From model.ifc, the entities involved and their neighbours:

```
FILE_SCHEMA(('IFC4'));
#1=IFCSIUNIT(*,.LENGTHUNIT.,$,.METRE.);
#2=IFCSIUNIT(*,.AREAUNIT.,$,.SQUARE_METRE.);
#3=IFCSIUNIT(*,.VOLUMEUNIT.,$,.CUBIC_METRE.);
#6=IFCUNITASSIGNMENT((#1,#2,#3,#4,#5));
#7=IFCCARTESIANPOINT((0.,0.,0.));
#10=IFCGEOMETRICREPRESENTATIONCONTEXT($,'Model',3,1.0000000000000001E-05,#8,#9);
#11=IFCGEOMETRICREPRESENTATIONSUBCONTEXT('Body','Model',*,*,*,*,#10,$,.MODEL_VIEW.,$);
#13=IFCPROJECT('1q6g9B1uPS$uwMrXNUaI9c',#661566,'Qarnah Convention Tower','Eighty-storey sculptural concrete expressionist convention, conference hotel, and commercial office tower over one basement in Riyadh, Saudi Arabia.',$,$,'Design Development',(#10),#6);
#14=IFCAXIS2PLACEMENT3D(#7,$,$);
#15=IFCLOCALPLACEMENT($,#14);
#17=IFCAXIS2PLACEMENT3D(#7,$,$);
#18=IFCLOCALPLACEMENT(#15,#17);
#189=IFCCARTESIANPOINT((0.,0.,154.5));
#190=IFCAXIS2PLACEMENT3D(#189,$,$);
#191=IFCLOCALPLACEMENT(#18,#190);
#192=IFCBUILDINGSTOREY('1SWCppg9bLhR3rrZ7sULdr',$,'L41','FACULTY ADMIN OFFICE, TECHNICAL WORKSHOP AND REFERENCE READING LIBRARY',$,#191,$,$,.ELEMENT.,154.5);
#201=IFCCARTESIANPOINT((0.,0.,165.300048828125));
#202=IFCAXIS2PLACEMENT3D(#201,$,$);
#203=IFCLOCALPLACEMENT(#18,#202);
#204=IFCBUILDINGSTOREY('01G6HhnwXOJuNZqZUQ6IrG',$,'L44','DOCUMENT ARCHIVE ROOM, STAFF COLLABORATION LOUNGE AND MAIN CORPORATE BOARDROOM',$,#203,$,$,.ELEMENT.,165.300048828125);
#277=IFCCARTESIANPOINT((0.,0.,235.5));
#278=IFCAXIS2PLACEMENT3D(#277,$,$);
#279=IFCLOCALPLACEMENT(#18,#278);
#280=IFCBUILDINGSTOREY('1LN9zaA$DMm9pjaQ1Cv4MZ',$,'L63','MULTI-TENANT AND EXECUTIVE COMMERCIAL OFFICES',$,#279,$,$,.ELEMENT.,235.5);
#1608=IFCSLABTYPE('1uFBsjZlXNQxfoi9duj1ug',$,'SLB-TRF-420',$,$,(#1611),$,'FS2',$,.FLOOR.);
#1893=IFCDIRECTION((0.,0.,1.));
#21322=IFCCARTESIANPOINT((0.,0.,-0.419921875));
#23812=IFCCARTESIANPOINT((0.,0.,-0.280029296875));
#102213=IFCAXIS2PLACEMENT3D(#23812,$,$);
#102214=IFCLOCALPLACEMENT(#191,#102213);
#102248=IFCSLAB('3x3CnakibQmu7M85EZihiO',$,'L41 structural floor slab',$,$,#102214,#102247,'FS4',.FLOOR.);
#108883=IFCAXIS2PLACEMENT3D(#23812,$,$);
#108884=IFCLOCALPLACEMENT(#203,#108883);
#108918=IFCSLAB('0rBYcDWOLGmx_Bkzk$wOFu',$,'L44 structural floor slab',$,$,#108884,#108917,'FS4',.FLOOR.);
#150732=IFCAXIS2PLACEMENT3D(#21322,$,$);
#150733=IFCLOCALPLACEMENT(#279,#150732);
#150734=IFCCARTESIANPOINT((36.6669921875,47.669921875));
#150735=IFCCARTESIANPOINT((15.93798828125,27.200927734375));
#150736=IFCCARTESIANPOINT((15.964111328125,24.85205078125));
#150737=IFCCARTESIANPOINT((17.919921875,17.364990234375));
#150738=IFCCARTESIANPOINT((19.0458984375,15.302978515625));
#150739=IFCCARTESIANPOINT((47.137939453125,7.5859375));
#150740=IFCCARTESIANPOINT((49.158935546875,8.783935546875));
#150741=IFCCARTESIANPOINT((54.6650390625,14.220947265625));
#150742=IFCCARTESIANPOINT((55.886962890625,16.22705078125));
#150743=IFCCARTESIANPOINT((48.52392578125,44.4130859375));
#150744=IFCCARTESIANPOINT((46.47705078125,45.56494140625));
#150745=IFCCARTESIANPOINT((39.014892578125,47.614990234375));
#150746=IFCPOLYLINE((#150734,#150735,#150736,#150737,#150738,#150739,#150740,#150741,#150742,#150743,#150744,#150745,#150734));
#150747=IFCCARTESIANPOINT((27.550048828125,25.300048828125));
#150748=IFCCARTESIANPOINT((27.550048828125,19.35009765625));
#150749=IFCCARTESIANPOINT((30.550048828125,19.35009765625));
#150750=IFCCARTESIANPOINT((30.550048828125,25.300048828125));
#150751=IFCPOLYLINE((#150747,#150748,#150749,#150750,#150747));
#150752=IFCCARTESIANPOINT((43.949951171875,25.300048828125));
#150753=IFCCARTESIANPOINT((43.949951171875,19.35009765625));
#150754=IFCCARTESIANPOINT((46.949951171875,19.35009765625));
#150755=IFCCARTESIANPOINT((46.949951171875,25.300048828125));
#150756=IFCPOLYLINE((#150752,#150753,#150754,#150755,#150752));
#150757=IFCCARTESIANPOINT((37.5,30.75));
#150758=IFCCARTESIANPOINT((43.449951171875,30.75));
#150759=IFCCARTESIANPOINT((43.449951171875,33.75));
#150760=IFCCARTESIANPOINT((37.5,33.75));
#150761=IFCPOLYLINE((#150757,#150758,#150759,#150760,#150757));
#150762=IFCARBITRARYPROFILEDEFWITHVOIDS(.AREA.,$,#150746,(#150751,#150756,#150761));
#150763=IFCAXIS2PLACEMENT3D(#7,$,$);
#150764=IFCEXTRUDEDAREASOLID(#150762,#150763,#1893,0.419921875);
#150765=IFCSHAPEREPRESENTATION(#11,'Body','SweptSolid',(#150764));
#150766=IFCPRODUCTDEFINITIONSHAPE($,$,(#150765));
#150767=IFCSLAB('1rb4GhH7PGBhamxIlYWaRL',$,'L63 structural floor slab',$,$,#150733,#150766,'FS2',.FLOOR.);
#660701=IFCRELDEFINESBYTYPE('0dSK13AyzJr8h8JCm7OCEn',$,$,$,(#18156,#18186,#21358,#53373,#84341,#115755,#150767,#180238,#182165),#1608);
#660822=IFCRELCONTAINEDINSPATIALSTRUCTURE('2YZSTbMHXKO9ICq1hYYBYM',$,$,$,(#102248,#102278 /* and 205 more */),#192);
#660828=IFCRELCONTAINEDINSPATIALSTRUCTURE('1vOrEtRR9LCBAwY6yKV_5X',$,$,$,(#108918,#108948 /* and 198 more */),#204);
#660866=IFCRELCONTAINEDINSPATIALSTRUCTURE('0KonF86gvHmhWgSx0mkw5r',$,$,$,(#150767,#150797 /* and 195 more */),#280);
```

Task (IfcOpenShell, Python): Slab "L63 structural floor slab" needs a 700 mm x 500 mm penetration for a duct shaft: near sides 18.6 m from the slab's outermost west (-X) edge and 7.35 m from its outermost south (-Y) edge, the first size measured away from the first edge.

```python
import numpy as np
import ifcopenshell
import ifcopenshell.api.feature
import ifcopenshell.api.geometry
import ifcopenshell.api.root
import ifcopenshell.geom
import ifcopenshell.util.placement
import ifcopenshell.util.representation
import ifcopenshell.util.shape
import ifcopenshell.util.unit

model = ifcopenshell.open("model.ifc")
unit_scale = ifcopenshell.util.unit.calculate_unit_scale(model)
settings = ifcopenshell.geom.settings()


def volume(element):
    """Net volume in cubic metres, openings subtracted."""
    shape = ifcopenshell.geom.create_shape(settings, element)
    return ifcopenshell.util.shape.get_volume(shape.geometry)


slab = model.by_id(150767)
before = volume(slab)

# Extent in the slab's own axes, in metres. The edges named are its -X and -Y sides.
slab_shape = ifcopenshell.geom.create_shape(settings, slab)
vertices = ifcopenshell.util.shape.get_vertices(slab_shape.geometry)
x_min, y_min, bottom = vertices.min(axis=0)
top = vertices[:, 2].max()

opening = ifcopenshell.api.root.create_entity(model, ifc_class="IfcOpeningElement", name="Duct shaft opening", predefined_type="OPENING")
context = ifcopenshell.util.representation.get_context(model, "Model", "Body", "MODEL_VIEW")
width, depth = 0.7, 0.5
outline = [(0.0, 0.0), (width, 0.0), (width, depth), (0.0, depth), (0.0, 0.0)]
# Overshoot both faces by 50 mm so the cut is clean.
shape = ifcopenshell.api.geometry.add_slab_representation(
    model, context=context, depth=top - bottom + 0.1, polyline=outline
)
ifcopenshell.api.geometry.assign_representation(model, product=opening, representation=shape)

matrix = ifcopenshell.util.placement.get_local_placement(slab.ObjectPlacement)
matrix[:, 3] = matrix @ np.append(np.array([x_min + 18.6, y_min + 7.35, bottom - 0.05]) / unit_scale, 1.0)
ifcopenshell.api.geometry.edit_object_placement(model, product=opening, matrix=matrix, is_si=False)
ifcopenshell.api.feature.add_feature(model, feature=opening, element=slab)

after = volume(slab)

print(f"slab volume {before:.3f} -> {after:.3f} m3")

model.write("model_rev.ifc")
```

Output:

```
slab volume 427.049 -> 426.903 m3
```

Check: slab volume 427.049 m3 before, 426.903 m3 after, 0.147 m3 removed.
